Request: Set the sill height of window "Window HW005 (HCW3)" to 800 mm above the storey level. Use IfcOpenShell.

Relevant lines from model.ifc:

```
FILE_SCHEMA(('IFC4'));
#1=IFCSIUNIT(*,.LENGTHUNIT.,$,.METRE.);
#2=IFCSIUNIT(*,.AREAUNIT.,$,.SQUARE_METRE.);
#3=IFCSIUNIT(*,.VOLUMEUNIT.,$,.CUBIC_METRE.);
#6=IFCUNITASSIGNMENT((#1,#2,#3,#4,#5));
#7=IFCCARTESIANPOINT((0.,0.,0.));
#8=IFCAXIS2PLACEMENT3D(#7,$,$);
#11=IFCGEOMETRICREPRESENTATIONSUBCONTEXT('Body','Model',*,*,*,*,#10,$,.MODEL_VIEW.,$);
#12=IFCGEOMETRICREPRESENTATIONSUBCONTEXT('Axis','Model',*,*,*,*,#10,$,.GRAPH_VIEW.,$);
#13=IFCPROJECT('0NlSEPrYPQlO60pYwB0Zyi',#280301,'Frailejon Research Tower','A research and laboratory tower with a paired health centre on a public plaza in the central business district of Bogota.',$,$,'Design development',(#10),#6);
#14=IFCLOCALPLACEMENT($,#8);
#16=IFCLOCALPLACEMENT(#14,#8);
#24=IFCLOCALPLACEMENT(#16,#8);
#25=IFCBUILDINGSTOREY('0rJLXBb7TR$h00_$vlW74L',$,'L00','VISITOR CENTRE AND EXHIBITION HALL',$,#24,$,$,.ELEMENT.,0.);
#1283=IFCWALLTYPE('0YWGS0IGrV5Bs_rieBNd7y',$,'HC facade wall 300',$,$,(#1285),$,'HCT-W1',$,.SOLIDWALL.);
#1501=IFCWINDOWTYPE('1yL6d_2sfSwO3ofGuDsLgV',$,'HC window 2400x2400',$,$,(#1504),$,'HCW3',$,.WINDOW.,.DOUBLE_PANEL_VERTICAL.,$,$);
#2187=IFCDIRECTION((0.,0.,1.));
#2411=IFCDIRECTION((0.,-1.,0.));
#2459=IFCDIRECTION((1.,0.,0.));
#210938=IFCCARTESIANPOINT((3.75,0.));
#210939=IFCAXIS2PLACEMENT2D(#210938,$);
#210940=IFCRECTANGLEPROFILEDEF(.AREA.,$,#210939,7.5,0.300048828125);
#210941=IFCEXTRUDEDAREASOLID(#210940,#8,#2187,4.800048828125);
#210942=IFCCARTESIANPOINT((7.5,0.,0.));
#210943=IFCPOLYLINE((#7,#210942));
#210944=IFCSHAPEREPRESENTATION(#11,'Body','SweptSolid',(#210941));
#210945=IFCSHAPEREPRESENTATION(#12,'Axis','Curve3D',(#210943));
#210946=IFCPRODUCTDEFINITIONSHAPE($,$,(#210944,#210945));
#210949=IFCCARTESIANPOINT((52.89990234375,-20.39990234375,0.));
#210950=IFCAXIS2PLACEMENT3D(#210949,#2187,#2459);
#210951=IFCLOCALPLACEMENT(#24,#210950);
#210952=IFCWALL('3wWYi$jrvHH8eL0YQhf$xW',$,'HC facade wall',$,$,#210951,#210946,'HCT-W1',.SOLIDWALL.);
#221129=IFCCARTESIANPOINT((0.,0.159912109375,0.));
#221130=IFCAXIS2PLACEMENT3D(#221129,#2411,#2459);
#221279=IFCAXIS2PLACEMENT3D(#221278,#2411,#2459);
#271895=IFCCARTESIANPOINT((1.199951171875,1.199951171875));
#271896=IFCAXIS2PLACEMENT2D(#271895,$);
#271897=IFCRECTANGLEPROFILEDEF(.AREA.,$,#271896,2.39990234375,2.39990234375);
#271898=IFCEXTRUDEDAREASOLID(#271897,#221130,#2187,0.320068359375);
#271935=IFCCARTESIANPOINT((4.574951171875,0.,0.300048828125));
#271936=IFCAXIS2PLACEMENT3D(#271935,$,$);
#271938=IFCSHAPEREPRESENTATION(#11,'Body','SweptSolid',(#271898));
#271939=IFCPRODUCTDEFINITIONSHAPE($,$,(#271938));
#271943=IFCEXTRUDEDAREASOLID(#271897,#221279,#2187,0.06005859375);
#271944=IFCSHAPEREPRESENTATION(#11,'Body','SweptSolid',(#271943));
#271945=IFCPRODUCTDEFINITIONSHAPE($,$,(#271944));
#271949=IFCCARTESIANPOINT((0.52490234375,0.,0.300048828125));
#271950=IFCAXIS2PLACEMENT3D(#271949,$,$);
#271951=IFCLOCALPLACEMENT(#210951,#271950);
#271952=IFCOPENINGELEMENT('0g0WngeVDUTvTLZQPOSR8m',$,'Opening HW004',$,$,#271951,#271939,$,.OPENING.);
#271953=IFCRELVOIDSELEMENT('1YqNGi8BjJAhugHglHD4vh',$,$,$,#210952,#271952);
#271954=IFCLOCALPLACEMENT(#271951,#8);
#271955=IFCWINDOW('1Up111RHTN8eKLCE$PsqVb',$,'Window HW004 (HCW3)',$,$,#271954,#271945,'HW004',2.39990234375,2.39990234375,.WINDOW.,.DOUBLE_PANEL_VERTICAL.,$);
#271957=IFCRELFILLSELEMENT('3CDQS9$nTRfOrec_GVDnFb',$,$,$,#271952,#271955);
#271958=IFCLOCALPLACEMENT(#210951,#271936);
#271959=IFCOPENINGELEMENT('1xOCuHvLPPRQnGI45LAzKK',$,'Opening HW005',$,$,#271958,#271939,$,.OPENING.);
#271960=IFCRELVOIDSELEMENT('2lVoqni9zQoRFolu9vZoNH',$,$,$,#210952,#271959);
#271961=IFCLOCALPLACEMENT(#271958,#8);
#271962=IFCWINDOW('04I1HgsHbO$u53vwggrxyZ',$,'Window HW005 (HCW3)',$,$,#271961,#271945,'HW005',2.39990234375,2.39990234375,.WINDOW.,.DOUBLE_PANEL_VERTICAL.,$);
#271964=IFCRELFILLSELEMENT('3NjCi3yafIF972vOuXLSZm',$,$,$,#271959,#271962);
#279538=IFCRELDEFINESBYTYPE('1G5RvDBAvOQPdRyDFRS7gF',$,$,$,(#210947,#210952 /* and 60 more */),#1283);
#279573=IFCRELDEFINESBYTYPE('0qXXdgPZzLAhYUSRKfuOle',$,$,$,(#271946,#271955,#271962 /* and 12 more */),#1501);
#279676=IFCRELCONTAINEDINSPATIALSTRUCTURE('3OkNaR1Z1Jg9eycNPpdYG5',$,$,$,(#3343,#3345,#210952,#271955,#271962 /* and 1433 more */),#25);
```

```python
import numpy as np
import ifcopenshell
import ifcopenshell.api.geometry
import ifcopenshell.geom
import ifcopenshell.util.element
import ifcopenshell.util.placement
import ifcopenshell.util.shape
import ifcopenshell.util.unit

model = ifcopenshell.open("model.ifc")
unit_scale = ifcopenshell.util.unit.calculate_unit_scale(model)

window = model.by_guid("04I1HgsHbO$u53vwggrxyZ")
opening = window.FillsVoids[0].RelatingOpeningElement
storey = ifcopenshell.util.element.get_container(window, ifc_class="IfcBuildingStorey")
level = ifcopenshell.util.placement.get_local_placement(storey.ObjectPlacement)[2, 3]

# The opening's origin need not be at the sill, so measure its lowest point.
shape = ifcopenshell.geom.create_shape(ifcopenshell.geom.settings(), opening)
bottom = ifcopenshell.util.shape.get_shape_bottom_elevation(shape, shape.geometry) / unit_scale
dz = level + 0.8 - bottom

shift = np.array([0.0, 0.0, dz])
# The window is placed relative to its opening, so it follows when the opening moves.
matrix = ifcopenshell.util.placement.get_local_placement(opening.ObjectPlacement)
matrix[:3, 3] += shift
ifcopenshell.api.geometry.edit_object_placement(
    model, product=opening, matrix=matrix, is_si=False, should_transform_children=True
)

print(f"moved by {dz * unit_scale:+.3f} m")

model.write("model-out.ifc")
```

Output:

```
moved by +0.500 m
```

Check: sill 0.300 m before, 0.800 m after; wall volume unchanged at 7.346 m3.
